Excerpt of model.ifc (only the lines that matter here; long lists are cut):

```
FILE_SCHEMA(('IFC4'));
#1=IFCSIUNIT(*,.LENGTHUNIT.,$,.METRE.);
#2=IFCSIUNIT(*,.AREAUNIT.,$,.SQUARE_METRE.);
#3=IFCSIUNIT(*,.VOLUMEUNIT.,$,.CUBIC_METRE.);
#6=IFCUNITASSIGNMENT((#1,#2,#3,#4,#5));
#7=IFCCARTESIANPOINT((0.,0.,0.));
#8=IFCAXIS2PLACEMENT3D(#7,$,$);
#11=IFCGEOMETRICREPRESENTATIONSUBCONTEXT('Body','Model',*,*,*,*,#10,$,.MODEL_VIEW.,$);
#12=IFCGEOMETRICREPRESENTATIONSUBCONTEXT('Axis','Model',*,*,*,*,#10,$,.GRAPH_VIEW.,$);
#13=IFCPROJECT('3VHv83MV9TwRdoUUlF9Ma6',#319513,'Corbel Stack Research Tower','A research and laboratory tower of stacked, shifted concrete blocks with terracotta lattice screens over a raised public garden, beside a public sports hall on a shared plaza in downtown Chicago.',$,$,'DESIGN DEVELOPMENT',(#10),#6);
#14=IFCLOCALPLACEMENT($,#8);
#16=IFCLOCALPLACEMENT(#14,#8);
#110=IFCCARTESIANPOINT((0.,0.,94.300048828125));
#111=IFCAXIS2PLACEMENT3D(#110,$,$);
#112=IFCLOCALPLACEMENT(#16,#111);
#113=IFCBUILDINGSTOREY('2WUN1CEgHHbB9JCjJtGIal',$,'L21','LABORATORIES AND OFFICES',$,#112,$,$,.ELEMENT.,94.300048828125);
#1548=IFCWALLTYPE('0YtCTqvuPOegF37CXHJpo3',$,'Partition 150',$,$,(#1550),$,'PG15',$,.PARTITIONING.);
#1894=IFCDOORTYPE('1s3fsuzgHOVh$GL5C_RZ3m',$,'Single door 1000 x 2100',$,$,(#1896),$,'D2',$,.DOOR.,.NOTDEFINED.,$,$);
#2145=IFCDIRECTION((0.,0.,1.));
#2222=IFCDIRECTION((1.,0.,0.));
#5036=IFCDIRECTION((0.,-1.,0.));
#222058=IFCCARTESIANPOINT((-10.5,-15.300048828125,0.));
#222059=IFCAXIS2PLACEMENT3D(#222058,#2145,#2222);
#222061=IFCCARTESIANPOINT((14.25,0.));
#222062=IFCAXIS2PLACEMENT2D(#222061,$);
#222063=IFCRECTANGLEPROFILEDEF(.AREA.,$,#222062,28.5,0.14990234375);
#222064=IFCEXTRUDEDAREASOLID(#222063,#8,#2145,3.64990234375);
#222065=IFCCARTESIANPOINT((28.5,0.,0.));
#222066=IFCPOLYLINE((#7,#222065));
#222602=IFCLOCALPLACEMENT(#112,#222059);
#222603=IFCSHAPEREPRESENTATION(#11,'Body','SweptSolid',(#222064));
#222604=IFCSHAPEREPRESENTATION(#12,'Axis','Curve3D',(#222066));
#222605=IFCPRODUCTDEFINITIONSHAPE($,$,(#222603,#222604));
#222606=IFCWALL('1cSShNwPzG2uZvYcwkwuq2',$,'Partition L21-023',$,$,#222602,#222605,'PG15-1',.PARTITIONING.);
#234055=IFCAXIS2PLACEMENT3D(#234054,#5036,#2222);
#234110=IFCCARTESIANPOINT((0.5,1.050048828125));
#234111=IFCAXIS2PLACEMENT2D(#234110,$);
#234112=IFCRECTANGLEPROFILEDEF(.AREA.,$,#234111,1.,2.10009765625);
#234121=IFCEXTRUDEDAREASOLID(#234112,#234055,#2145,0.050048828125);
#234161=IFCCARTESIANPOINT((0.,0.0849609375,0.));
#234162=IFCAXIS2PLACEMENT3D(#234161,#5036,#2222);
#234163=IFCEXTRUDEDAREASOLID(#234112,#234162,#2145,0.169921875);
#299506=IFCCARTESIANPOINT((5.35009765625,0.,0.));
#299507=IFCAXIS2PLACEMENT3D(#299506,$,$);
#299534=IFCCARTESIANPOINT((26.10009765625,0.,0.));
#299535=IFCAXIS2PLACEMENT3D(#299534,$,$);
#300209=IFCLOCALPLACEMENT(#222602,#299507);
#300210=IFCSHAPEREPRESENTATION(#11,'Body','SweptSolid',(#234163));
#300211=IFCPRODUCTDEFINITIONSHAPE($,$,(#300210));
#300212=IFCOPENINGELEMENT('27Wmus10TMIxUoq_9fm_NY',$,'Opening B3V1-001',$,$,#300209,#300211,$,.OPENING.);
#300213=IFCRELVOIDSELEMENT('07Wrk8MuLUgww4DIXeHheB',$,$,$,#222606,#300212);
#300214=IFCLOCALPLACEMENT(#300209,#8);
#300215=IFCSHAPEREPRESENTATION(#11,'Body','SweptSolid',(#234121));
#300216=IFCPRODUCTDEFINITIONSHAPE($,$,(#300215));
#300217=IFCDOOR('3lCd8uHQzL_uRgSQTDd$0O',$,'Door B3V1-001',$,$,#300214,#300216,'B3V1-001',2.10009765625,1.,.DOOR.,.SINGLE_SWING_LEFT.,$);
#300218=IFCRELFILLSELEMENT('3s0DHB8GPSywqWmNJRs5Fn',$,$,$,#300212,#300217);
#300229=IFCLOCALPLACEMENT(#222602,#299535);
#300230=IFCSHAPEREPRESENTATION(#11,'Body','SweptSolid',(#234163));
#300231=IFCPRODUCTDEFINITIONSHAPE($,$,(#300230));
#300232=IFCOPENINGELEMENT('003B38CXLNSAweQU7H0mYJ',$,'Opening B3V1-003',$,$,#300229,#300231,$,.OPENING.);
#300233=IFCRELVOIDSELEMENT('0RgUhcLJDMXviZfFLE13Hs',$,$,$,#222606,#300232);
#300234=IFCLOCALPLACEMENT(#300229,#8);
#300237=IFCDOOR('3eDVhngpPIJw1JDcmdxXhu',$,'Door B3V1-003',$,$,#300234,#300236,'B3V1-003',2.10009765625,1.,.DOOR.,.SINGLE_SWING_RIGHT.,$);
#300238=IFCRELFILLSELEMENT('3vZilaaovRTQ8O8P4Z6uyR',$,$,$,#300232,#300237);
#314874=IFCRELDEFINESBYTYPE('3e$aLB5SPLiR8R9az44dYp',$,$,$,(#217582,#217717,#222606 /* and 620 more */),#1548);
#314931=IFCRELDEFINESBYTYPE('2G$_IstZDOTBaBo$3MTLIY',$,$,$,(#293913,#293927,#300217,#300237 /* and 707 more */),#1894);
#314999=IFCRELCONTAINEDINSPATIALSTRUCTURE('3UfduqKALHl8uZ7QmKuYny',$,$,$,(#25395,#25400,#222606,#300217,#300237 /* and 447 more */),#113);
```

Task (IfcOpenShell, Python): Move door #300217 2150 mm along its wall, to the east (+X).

```python
import ifcopenshell
import ifcopenshell.api.geometry
import ifcopenshell.util.placement
import ifcopenshell.util.unit

model = ifcopenshell.open("model.ifc")
unit_scale = ifcopenshell.util.unit.calculate_unit_scale(model)

door = model.by_id(300217)
opening = door.FillsVoids[0].RelatingOpeningElement
wall = opening.VoidsElements[0].RelatingBuildingElement

wall_matrix = ifcopenshell.util.placement.get_local_placement(wall.ObjectPlacement)
shift = wall_matrix[:3, 0] * 2.15 / unit_scale
before = ifcopenshell.util.placement.get_local_placement(door.ObjectPlacement)[:3, 3].copy()

# The door is placed relative to its opening, so it follows when the opening moves.
matrix = ifcopenshell.util.placement.get_local_placement(opening.ObjectPlacement)
matrix[:3, 3] += shift
ifcopenshell.api.geometry.edit_object_placement(
    model, product=opening, matrix=matrix, is_si=False, should_transform_children=True
)

after = ifcopenshell.util.placement.get_local_placement(door.ObjectPlacement)[:3, 3]
print("door moved by", (after - before).round(3) + 0.0)

model.write("model_edited.ifc")
```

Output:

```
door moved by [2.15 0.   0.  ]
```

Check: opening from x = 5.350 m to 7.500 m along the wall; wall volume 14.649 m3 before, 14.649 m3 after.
